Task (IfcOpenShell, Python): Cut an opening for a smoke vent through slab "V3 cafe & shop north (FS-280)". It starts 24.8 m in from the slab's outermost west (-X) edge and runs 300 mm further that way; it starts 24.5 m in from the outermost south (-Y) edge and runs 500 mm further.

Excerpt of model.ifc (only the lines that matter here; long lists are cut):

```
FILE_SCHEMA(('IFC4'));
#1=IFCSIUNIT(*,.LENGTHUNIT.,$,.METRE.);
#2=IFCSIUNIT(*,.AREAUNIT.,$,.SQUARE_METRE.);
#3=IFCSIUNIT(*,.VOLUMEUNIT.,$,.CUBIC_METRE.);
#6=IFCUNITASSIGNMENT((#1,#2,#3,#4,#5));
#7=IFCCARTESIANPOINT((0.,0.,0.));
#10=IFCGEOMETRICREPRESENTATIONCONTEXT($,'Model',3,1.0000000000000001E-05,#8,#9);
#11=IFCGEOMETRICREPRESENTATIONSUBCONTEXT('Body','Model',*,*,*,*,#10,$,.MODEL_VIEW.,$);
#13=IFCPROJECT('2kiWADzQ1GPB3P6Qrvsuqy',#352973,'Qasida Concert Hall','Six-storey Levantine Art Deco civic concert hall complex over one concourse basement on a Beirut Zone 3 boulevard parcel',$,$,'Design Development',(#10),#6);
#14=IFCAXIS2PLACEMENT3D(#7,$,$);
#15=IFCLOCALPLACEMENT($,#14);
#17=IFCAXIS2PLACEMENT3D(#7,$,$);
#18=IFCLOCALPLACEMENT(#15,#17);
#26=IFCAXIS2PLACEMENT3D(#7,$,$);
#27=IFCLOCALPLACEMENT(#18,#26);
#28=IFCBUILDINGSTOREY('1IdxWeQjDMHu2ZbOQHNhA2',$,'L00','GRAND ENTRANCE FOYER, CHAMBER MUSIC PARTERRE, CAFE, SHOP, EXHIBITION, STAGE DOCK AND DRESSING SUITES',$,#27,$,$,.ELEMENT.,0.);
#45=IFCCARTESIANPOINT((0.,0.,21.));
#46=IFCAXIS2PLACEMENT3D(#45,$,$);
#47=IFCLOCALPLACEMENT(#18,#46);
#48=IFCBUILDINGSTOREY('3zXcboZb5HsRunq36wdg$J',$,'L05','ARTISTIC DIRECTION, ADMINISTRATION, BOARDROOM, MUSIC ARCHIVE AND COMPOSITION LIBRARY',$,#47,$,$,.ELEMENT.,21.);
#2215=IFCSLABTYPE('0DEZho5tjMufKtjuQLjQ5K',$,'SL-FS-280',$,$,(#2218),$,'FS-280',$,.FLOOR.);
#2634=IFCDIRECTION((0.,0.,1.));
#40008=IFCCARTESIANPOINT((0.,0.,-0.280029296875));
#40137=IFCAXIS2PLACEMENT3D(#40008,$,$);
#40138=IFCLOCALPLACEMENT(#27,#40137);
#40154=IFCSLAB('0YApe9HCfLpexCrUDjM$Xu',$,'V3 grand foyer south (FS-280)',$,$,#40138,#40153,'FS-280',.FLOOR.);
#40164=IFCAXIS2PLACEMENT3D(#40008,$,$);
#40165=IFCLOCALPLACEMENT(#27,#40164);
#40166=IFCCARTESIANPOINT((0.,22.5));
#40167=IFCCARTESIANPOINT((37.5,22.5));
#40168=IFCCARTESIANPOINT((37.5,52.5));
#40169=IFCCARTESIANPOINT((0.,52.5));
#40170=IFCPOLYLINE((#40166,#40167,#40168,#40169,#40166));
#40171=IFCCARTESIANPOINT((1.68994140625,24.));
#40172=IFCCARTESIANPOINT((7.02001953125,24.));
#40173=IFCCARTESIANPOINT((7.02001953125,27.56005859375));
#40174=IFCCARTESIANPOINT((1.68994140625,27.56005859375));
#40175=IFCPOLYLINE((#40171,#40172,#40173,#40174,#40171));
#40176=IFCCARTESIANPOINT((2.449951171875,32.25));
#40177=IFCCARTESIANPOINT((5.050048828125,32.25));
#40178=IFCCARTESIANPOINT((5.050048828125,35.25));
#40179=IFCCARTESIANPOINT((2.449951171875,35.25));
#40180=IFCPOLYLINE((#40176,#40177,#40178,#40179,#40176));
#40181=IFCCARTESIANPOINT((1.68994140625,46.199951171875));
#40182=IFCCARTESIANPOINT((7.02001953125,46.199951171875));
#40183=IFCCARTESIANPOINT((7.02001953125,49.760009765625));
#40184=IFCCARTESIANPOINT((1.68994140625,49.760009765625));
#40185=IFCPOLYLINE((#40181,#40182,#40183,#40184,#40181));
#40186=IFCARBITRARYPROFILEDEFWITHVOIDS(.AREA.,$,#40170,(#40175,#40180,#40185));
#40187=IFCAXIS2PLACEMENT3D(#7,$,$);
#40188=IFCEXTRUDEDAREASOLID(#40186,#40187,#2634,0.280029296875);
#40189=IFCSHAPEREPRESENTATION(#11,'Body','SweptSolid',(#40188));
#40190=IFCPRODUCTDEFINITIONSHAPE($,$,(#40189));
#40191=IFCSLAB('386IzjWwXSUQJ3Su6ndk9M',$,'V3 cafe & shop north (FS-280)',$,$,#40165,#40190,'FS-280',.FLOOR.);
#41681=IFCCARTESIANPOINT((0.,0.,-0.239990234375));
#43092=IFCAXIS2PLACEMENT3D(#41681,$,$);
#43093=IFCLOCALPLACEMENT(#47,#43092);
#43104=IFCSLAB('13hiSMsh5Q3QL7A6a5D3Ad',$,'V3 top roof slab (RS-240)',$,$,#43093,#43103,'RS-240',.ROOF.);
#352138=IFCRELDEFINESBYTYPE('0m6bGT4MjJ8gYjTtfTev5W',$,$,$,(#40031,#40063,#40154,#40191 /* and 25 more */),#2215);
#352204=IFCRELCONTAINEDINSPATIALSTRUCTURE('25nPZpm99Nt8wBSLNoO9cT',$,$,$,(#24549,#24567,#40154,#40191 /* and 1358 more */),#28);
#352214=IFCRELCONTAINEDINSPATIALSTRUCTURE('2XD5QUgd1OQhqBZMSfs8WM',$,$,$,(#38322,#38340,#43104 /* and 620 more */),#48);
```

```python
import numpy as np
import ifcopenshell
import ifcopenshell.api.feature
import ifcopenshell.api.geometry
import ifcopenshell.api.root
import ifcopenshell.geom
import ifcopenshell.util.placement
import ifcopenshell.util.representation
import ifcopenshell.util.shape
import ifcopenshell.util.unit

model = ifcopenshell.open("model.ifc")
unit_scale = ifcopenshell.util.unit.calculate_unit_scale(model)
settings = ifcopenshell.geom.settings()


def volume(element):
    """Net volume in cubic metres, openings subtracted."""
    shape = ifcopenshell.geom.create_shape(settings, element)
    return ifcopenshell.util.shape.get_volume(shape.geometry)


slab = model.by_id(40191)
before = volume(slab)

# Extent in the slab's own axes, in metres. The edges named are its -X and -Y sides.
slab_shape = ifcopenshell.geom.create_shape(settings, slab)
vertices = ifcopenshell.util.shape.get_vertices(slab_shape.geometry)
x_min, y_min, bottom = vertices.min(axis=0)
top = vertices[:, 2].max()

opening = ifcopenshell.api.root.create_entity(model, ifc_class="IfcOpeningElement", name="Smoke vent opening", predefined_type="OPENING")
context = ifcopenshell.util.representation.get_context(model, "Model", "Body", "MODEL_VIEW")
width, depth = 0.3, 0.5
outline = [(0.0, 0.0), (width, 0.0), (width, depth), (0.0, depth), (0.0, 0.0)]
# Overshoot both faces by 50 mm so the cut is clean.
shape = ifcopenshell.api.geometry.add_slab_representation(
    model, context=context, depth=top - bottom + 0.1, polyline=outline
)
ifcopenshell.api.geometry.assign_representation(model, product=opening, representation=shape)

matrix = ifcopenshell.util.placement.get_local_placement(slab.ObjectPlacement)
matrix[:, 3] = matrix @ np.append(np.array([x_min + 24.8, y_min + 24.5, bottom - 0.05]) / unit_scale, 1.0)
ifcopenshell.api.geometry.edit_object_placement(model, product=opening, matrix=matrix, is_si=False)
ifcopenshell.api.feature.add_feature(model, feature=opening, element=slab)

after = volume(slab)

print(f"slab volume {before:.3f} -> {after:.3f} m3")

model.write("model_v2.ifc")
```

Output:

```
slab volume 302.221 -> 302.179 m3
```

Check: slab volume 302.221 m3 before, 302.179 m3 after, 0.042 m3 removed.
